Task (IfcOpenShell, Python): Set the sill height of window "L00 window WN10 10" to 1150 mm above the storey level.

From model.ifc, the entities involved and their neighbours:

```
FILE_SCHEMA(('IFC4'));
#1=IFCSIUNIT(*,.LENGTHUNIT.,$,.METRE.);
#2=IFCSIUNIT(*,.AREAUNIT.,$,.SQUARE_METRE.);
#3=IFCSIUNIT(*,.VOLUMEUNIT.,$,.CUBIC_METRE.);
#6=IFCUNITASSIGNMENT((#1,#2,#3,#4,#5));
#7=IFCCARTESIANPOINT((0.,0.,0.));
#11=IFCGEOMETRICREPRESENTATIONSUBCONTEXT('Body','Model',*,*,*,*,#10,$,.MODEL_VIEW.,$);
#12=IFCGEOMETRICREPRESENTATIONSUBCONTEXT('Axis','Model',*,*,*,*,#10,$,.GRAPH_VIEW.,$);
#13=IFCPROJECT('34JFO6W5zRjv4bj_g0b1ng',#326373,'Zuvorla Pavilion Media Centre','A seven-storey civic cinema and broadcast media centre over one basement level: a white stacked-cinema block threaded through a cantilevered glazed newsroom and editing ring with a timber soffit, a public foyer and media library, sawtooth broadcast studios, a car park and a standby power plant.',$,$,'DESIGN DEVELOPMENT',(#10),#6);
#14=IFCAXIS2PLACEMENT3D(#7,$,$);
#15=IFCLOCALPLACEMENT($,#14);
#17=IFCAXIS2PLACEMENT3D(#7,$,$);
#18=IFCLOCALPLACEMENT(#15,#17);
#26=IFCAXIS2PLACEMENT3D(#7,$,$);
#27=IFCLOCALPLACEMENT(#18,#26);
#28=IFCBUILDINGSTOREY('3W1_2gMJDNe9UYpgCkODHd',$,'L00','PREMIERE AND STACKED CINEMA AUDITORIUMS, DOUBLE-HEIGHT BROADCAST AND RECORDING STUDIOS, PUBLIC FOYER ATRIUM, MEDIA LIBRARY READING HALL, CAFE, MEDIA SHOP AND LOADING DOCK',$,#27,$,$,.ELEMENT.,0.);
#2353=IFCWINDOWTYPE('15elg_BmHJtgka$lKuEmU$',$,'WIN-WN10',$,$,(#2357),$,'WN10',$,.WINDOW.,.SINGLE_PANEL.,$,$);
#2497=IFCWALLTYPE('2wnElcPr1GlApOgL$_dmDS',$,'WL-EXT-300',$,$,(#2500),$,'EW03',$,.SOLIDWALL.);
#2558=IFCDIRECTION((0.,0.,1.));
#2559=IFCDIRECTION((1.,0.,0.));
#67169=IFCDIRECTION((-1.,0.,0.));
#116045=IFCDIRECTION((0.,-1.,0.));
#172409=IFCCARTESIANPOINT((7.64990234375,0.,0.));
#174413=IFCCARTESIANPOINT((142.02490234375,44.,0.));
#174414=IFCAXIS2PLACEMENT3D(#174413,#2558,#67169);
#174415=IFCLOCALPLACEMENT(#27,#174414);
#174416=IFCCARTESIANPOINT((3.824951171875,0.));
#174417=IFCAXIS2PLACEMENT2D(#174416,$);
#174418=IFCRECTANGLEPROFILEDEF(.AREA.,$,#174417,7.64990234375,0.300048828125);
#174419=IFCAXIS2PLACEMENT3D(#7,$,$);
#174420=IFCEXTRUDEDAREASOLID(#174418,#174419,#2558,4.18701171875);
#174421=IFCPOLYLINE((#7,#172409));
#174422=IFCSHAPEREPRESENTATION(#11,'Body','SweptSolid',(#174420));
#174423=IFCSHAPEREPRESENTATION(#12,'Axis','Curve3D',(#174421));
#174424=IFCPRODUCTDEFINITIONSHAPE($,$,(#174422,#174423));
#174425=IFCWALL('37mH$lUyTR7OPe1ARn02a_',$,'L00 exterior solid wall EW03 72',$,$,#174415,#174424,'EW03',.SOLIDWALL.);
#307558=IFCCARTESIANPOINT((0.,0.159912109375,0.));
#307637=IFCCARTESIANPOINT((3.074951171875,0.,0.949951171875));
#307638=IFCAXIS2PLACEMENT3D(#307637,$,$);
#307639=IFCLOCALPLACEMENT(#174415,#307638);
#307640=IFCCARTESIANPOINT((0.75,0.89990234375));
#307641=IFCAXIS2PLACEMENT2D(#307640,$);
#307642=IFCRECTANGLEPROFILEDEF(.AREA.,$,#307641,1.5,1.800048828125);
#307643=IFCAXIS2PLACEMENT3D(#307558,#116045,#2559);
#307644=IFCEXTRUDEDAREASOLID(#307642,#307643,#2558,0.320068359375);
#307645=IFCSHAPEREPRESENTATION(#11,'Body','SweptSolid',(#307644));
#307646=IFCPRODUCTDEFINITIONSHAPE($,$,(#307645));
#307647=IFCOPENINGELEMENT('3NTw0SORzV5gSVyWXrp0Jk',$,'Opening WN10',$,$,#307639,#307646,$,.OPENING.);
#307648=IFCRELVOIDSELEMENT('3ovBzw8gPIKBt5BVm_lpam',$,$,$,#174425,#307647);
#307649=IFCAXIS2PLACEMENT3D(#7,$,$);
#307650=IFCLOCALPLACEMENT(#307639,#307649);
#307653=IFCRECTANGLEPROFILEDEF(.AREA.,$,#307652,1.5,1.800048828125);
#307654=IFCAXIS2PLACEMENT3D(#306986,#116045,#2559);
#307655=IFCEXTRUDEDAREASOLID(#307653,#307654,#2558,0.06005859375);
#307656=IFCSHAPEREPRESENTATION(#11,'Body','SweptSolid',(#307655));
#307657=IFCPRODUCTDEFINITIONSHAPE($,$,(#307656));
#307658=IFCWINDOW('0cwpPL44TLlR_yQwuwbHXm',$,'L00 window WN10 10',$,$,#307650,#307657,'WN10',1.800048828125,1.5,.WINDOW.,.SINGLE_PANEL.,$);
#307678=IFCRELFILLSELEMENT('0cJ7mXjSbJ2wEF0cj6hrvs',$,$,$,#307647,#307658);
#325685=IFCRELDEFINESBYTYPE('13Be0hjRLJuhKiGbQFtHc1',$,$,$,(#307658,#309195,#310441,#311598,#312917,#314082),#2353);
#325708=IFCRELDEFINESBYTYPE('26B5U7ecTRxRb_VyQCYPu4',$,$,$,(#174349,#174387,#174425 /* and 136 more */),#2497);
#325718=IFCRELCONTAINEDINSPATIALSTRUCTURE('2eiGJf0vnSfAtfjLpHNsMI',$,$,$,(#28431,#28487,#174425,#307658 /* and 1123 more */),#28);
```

```python
import numpy as np
import ifcopenshell
import ifcopenshell.api.geometry
import ifcopenshell.geom
import ifcopenshell.util.element
import ifcopenshell.util.placement
import ifcopenshell.util.shape
import ifcopenshell.util.unit

model = ifcopenshell.open("model.ifc")
unit_scale = ifcopenshell.util.unit.calculate_unit_scale(model)

window = model.by_id(307658)
opening = window.FillsVoids[0].RelatingOpeningElement
storey = ifcopenshell.util.element.get_container(window, ifc_class="IfcBuildingStorey")
level = ifcopenshell.util.placement.get_local_placement(storey.ObjectPlacement)[2, 3]

# The opening's origin need not be at the sill, so measure its lowest point.
shape = ifcopenshell.geom.create_shape(ifcopenshell.geom.settings(), opening)
bottom = ifcopenshell.util.shape.get_shape_bottom_elevation(shape, shape.geometry) / unit_scale
dz = level + 1.15 / unit_scale - bottom

shift = np.array([0.0, 0.0, dz])
# The window is placed relative to its opening, so it follows when the opening moves.
matrix = ifcopenshell.util.placement.get_local_placement(opening.ObjectPlacement)
matrix[:3, 3] += shift
ifcopenshell.api.geometry.edit_object_placement(
    model, product=opening, matrix=matrix, is_si=False, should_transform_children=True
)

print(f"moved by {dz * unit_scale:+.3f} m")

model.write("model_rev.ifc")
```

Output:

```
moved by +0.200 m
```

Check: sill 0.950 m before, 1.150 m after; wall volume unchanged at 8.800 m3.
